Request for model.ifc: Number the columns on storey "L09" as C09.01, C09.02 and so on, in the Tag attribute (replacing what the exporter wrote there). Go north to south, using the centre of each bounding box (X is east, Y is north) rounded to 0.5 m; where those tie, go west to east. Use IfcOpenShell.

First a look at what the model holds.

```python
import ifcopenshell
import ifcopenshell.util.element
import ifcopenshell.util.placement

model = ifcopenshell.open("model.ifc")
print(model.schema)
storey = next(s for s in model.by_type("IfcBuildingStorey") if s.Name == "L09")
columns = [e for e in ifcopenshell.util.element.get_decomposition(storey) if e.is_a("IfcColumn")]
for e in sorted(columns, key=lambda e: e.id()):
    origin = ifcopenshell.util.placement.get_local_placement(e.ObjectPlacement)[:3, 3]
    print(e.id(), e.Tag, e.Name, origin.round(2) + 0.0, sep=" | ")
```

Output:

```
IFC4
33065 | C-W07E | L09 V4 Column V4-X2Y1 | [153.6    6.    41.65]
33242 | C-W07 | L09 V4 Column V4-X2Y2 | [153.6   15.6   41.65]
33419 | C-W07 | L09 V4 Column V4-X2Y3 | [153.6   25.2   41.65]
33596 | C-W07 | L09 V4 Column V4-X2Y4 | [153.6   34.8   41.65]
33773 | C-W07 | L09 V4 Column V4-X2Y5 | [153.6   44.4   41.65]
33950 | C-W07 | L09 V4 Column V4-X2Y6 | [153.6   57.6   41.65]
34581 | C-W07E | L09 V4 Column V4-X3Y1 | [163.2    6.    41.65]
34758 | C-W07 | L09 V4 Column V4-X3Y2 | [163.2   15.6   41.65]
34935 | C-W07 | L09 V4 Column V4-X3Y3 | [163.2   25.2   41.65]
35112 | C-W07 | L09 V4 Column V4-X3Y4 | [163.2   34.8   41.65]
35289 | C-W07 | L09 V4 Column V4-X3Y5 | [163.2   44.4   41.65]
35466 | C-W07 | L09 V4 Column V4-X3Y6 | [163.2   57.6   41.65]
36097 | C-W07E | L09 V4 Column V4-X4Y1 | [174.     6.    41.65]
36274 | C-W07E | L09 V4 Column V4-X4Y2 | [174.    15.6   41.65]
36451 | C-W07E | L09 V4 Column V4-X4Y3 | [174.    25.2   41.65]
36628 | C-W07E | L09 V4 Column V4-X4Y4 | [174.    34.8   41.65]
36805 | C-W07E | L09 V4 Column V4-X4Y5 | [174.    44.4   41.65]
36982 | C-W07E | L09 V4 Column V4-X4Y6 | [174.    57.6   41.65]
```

```python
import ifcopenshell
import ifcopenshell.geom
import ifcopenshell.util.element
import ifcopenshell.util.shape

model = ifcopenshell.open("model.ifc")
settings = ifcopenshell.geom.settings()
settings.set("use-world-coords", True)


def centre(element):
    shape = ifcopenshell.geom.create_shape(settings, element)
    return ifcopenshell.util.shape.get_bbox_centroid(shape.geometry)


storey = next(s for s in model.by_type("IfcBuildingStorey") if s.Name == "L09")
columns = [e for e in ifcopenshell.util.element.get_decomposition(storey) if e.is_a("IfcColumn")]

# Insertion points can sit at a corner or the storey origin, so sort by the geometry (in metres).
centres = {e: centre(e) for e in columns}
columns.sort(key=lambda e: (-round(centres[e][1] / 0.5), centres[e][0]))

for i, e in enumerate(columns, start=1):
    number = f"C09.{i:02d}"
    e.Tag = number
    print(e.id(), number)

model.write("model-out.ifc")
```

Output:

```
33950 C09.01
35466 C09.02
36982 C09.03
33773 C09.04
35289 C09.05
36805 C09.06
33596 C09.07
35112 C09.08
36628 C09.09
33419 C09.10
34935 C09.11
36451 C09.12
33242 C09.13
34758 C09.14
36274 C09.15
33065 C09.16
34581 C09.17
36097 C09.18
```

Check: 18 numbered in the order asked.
